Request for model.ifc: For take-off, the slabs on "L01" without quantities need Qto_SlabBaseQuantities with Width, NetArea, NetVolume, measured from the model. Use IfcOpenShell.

First a look at what the model holds.

```python
import ifcopenshell
import ifcopenshell.util.element
import ifcopenshell.util.unit

model = ifcopenshell.open("model.ifc")
print(model.schema)
for unit_type in ("LENGTHUNIT", "AREAUNIT", "VOLUMEUNIT"):
    print(unit_type, ifcopenshell.util.unit.calculate_unit_scale(model, unit_type))
storey = next(s for s in model.by_type("IfcBuildingStorey") if s.Name == "L01")
slabs = [e for e in ifcopenshell.util.element.get_decomposition(storey) if e.is_a("IfcSlab")]
for e in sorted(slabs, key=lambda e: e.id()):
    print(e.id(), e.is_a(), e.Name, list(ifcopenshell.util.element.get_psets(e, qtos_only=True)), sep=" | ")
```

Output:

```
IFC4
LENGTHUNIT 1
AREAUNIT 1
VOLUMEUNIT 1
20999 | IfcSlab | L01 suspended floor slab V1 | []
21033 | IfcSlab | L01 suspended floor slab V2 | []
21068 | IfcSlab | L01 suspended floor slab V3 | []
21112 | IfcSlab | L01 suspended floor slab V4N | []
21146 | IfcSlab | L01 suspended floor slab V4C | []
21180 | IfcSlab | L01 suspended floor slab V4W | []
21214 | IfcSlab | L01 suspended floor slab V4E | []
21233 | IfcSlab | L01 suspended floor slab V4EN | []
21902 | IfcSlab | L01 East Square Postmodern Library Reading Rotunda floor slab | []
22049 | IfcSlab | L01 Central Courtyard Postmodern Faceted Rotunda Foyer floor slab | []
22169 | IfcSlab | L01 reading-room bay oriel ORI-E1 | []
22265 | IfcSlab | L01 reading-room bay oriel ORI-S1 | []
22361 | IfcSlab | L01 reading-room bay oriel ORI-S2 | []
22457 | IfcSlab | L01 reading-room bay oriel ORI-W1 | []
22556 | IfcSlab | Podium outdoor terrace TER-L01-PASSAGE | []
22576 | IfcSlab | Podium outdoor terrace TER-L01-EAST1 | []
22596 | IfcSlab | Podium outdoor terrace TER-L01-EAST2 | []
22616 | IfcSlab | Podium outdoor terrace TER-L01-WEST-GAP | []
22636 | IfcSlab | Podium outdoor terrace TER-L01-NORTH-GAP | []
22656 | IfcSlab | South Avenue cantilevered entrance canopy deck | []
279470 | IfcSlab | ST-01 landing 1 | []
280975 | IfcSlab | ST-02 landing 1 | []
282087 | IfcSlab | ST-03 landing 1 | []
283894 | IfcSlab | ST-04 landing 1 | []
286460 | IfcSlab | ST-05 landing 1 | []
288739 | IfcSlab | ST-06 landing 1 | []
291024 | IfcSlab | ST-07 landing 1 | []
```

```python
import ifcopenshell
import ifcopenshell.api.pset
import ifcopenshell.geom
import ifcopenshell.util.element
import ifcopenshell.util.shape
import ifcopenshell.util.unit

model = ifcopenshell.open("model.ifc")
unit_scale = ifcopenshell.util.unit.calculate_unit_scale(model)
area_scale = ifcopenshell.util.unit.calculate_unit_scale(model, "AREAUNIT")
volume_scale = ifcopenshell.util.unit.calculate_unit_scale(model, "VOLUMEUNIT")
settings = ifcopenshell.geom.settings()

storey = next(s for s in model.by_type("IfcBuildingStorey") if s.Name == "L01")
slabs = [e for e in ifcopenshell.util.element.get_decomposition(storey) if e.is_a("IfcSlab")]

for e in sorted(slabs, key=lambda e: e.id()):
    if ifcopenshell.util.element.get_psets(e, qtos_only=True, should_inherit=False):
        continue
    # Geometry comes back in metres, in the element's own axes.
    shape = ifcopenshell.geom.create_shape(settings, e)
    values = {
        "Width": ifcopenshell.util.shape.get_z(shape.geometry) / unit_scale,
        "NetArea": ifcopenshell.util.shape.get_footprint_area(shape.geometry) / area_scale,
        "NetVolume": ifcopenshell.util.shape.get_volume(shape.geometry) / volume_scale,
    }
    qto = ifcopenshell.api.pset.add_qto(model, product=e, name="Qto_SlabBaseQuantities")
    ifcopenshell.api.pset.edit_qto(model, qto=qto, properties=values)
    print(e.id(), {k: round(v, 3) for k, v in values.items()})

model.write("model-out.ifc")
```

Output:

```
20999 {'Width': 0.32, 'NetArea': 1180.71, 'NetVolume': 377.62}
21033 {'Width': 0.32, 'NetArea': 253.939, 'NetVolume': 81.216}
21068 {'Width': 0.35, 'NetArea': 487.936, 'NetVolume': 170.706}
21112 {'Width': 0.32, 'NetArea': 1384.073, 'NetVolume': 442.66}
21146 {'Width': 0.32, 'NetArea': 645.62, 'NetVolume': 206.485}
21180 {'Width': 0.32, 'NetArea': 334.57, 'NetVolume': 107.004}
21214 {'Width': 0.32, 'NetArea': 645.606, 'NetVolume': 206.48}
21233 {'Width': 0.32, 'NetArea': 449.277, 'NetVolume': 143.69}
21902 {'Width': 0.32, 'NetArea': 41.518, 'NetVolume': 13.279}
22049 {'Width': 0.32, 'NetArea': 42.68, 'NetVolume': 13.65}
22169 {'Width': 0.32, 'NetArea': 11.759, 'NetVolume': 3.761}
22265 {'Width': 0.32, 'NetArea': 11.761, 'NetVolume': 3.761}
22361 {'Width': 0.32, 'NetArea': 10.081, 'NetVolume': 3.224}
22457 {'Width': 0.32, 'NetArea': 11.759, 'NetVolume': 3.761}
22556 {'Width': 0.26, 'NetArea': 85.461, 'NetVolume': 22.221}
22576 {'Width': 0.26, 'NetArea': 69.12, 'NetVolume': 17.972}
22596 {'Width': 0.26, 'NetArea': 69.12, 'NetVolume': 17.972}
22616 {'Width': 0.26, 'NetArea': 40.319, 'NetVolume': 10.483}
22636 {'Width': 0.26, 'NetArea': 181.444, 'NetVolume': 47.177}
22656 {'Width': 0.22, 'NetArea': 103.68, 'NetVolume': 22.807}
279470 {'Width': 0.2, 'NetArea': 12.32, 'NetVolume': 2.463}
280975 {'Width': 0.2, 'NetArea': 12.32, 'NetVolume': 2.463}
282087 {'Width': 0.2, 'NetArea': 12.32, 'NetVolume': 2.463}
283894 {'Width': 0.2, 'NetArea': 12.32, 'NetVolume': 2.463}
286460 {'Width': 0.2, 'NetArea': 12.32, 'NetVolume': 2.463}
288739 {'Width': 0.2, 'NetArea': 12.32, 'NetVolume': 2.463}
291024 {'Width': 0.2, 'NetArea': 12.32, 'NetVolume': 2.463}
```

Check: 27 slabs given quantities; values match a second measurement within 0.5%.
